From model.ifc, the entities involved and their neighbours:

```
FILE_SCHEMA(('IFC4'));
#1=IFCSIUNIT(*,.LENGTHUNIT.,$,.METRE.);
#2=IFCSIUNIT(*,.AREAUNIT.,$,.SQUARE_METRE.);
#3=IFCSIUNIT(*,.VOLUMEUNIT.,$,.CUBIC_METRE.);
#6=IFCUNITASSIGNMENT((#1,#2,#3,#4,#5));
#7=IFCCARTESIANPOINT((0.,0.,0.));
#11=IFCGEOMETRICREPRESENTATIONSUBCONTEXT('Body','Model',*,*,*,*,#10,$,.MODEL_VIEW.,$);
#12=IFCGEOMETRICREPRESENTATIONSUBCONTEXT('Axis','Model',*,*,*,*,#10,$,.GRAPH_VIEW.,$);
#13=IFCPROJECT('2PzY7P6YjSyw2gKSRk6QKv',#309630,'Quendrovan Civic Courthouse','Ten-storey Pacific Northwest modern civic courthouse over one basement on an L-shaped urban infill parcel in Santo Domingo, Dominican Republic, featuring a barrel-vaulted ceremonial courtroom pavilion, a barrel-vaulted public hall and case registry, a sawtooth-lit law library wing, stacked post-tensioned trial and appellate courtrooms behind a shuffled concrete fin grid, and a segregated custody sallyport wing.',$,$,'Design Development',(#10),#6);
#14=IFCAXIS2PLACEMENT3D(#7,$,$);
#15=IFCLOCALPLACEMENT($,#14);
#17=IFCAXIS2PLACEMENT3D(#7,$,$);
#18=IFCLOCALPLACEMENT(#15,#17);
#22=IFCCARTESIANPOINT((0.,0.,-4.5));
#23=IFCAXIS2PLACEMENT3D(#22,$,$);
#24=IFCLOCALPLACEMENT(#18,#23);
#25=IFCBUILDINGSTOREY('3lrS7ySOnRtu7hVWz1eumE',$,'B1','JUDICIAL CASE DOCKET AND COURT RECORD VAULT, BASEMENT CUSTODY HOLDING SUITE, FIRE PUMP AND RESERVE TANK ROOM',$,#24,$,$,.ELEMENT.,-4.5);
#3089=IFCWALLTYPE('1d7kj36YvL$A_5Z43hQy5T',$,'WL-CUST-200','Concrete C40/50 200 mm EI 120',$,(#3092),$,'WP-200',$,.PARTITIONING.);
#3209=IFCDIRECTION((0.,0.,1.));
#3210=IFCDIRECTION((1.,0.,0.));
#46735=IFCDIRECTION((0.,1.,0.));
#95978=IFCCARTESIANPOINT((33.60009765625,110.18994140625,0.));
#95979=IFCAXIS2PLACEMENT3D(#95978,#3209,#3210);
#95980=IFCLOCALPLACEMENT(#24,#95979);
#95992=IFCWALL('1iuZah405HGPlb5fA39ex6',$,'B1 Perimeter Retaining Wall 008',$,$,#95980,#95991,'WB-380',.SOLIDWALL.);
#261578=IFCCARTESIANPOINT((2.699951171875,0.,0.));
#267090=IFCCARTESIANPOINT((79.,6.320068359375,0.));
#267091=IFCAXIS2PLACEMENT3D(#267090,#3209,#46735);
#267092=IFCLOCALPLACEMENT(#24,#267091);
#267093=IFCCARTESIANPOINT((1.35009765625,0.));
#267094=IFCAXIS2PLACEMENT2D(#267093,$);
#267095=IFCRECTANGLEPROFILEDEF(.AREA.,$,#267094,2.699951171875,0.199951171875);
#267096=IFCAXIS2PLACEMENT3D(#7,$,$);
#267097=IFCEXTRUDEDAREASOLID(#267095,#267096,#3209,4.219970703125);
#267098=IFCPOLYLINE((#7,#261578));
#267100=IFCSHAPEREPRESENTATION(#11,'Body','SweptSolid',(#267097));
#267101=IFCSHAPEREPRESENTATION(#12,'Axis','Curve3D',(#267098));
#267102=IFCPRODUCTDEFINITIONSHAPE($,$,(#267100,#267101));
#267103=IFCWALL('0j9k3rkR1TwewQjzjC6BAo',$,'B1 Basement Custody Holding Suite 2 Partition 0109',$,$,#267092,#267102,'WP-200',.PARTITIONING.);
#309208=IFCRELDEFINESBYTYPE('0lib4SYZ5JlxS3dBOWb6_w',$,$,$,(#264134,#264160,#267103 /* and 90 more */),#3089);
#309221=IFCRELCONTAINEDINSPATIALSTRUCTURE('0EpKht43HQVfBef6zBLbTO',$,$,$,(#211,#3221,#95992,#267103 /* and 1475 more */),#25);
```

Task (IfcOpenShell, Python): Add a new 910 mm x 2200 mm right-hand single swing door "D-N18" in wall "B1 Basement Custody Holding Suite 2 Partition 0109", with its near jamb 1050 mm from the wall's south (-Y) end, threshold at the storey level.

```python
import numpy as np
import ifcopenshell
import ifcopenshell.api.feature
import ifcopenshell.api.geometry
import ifcopenshell.api.root
import ifcopenshell.api.spatial
import ifcopenshell.geom
import ifcopenshell.util.element
import ifcopenshell.util.placement
import ifcopenshell.util.representation
import ifcopenshell.util.shape
import ifcopenshell.util.unit

model = ifcopenshell.open("model.ifc")
unit_scale = ifcopenshell.util.unit.calculate_unit_scale(model)
settings = ifcopenshell.geom.settings()


def volume(element):
    """Net volume in cubic metres, openings subtracted."""
    shape = ifcopenshell.geom.create_shape(settings, element)
    return ifcopenshell.util.shape.get_volume(shape.geometry)


wall = model.by_guid("0j9k3rkR1TwewQjzjC6BAo")
storey = ifcopenshell.util.element.get_container(wall, ifc_class="IfcBuildingStorey")
context = ifcopenshell.util.representation.get_context(model, "Model", "Body", "MODEL_VIEW")
before = volume(wall)

width, height, from_end, sill = 0.91, 2.2, 1.05, 0.0  # metres

# The wall runs along its own X axis, and the end named is its -X end.
wall_shape = ifcopenshell.geom.create_shape(settings, wall)
x, y, z = ifcopenshell.util.shape.get_vertices(wall_shape.geometry).T
start = x.min() + from_end
face, thickness = float(y.min()), float(y.max() - y.min())
wall_matrix = ifcopenshell.util.placement.get_local_placement(wall.ObjectPlacement)
level = ifcopenshell.util.placement.get_local_placement(storey.ObjectPlacement)[2, 3]


def in_wall(x, y):
    """Placement at x, y metres in the wall's axes, at sill height."""
    matrix = wall_matrix.copy()
    matrix[:, 3] = wall_matrix @ np.array([x / unit_scale, y / unit_scale, 0.0, 1.0])
    matrix[2, 3] = level + sill / unit_scale
    return matrix


# Opening: a box that overshoots both wall faces by 50 mm.
opening = ifcopenshell.api.root.create_entity(model, ifc_class="IfcOpeningElement", predefined_type="OPENING")
box = ifcopenshell.api.geometry.add_wall_representation(
    model, context=context, length=width, height=height, thickness=thickness + 0.1
)
ifcopenshell.api.geometry.assign_representation(model, product=opening, representation=box)
ifcopenshell.api.geometry.edit_object_placement(model, product=opening, matrix=in_wall(start, face - 0.05), is_si=False)
ifcopenshell.api.feature.add_feature(model, feature=opening, element=wall)

door = ifcopenshell.api.root.create_entity(model, ifc_class="IfcDoor", name="D-N18", predefined_type="DOOR")
door.OverallWidth, door.OverallHeight = width / unit_scale, height / unit_scale
door.OperationType = "SINGLE_SWING_RIGHT"
body = ifcopenshell.api.geometry.add_door_representation(
    model,
    context=context,
    overall_width=door.OverallWidth,
    overall_height=door.OverallHeight,
    operation_type="SINGLE_SWING_RIGHT",
    lining_properties={"LiningDepth": thickness / unit_scale, "ThresholdDepth": thickness / unit_scale},
)
ifcopenshell.api.geometry.assign_representation(model, product=door, representation=body)
ifcopenshell.api.spatial.assign_container(model, products=[door], relating_structure=storey)
ifcopenshell.api.feature.add_filling(model, opening=opening, element=door)

# The lining spans the wall, so the door starts at the wall face.
ifcopenshell.api.geometry.edit_object_placement(model, product=door, matrix=in_wall(start, face), is_si=False)

after = volume(wall)

print(f"wall volume {before:.3f} -> {after:.3f} m3")

model.write("model-out.ifc")
```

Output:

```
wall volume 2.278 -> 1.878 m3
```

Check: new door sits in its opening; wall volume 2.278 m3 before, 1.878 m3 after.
